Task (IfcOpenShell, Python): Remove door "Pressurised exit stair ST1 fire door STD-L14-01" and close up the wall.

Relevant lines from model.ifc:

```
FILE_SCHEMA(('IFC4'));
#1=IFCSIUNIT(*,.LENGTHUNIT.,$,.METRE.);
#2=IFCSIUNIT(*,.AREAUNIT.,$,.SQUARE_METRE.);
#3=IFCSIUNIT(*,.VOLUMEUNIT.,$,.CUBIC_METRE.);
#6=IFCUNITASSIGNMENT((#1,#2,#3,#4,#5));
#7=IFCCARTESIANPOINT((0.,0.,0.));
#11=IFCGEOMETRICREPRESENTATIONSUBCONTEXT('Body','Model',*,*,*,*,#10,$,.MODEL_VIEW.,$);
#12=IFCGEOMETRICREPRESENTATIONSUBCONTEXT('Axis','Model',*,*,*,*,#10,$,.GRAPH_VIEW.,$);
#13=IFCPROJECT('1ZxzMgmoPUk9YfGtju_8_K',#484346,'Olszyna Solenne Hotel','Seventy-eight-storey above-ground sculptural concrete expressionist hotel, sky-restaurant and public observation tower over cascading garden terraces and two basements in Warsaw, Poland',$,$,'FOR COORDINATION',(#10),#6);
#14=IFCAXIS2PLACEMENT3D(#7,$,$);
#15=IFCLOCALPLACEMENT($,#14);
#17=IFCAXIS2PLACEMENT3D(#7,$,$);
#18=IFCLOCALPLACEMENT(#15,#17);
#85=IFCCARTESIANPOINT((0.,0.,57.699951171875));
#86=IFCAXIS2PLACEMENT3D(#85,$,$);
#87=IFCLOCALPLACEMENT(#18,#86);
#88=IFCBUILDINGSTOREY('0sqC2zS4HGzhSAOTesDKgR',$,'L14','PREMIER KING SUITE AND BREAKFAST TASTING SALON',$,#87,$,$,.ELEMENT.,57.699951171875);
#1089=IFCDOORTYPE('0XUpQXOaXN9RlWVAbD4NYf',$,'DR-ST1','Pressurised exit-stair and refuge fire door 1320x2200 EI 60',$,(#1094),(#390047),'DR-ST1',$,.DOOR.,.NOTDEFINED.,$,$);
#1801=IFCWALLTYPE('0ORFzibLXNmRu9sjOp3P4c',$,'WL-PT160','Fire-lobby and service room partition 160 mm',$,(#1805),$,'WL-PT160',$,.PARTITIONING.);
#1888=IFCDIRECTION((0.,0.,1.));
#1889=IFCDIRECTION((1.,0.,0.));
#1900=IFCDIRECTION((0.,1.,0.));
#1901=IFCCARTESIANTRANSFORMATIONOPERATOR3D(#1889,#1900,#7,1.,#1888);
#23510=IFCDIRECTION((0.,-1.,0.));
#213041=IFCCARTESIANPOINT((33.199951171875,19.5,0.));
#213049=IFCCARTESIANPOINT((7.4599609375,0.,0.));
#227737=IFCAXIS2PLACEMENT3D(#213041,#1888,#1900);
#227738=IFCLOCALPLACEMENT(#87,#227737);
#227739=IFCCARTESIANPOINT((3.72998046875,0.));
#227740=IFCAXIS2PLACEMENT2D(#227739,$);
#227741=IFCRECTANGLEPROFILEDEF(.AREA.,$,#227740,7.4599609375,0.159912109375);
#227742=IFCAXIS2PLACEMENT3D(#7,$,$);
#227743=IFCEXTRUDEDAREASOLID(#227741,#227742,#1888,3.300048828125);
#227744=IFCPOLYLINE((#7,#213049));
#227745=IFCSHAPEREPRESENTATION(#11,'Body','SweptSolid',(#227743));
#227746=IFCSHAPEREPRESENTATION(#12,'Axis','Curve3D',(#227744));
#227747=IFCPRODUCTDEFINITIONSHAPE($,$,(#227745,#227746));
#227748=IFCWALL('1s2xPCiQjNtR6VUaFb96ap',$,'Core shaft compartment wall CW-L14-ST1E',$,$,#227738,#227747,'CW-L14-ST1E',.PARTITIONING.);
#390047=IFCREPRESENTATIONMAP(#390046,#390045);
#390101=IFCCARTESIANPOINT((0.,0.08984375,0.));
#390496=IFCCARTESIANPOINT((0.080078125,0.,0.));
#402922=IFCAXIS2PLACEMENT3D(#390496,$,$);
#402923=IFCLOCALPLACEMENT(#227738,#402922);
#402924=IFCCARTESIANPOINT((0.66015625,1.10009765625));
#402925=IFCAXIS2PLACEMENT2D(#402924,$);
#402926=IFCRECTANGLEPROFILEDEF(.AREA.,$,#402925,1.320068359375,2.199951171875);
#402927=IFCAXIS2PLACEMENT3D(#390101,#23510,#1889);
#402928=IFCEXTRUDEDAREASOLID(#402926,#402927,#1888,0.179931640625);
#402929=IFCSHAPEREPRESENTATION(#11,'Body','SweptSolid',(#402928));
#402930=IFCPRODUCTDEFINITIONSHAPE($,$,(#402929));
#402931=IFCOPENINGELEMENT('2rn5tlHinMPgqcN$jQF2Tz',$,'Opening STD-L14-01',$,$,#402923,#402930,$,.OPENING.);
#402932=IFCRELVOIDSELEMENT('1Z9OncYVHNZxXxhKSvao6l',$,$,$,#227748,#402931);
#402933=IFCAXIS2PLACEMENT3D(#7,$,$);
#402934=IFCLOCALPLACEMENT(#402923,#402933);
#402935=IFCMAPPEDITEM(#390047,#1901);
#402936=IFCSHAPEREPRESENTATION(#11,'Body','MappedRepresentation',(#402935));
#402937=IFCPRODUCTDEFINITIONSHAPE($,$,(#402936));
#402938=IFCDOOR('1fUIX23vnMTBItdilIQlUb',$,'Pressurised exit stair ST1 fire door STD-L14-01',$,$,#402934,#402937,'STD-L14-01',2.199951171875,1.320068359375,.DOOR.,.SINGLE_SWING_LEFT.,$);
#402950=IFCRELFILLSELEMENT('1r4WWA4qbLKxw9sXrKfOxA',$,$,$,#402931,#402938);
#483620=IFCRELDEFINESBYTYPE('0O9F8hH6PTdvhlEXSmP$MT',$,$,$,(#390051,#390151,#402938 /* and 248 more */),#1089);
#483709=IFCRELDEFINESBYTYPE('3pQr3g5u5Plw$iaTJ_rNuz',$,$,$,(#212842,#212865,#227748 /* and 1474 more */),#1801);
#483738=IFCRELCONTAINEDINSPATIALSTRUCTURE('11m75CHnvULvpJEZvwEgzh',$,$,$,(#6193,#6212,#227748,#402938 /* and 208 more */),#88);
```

```python
import ifcopenshell
import ifcopenshell.api.feature
import ifcopenshell.api.root
import ifcopenshell.geom
import ifcopenshell.util.shape

model = ifcopenshell.open("model.ifc")
settings = ifcopenshell.geom.settings()


def volume(element):
    """Net volume in cubic metres, openings subtracted."""
    shape = ifcopenshell.geom.create_shape(settings, element)
    return ifcopenshell.util.shape.get_volume(shape.geometry)


door = model.by_guid("1fUIX23vnMTBItdilIQlUb")
opening = door.FillsVoids[0].RelatingOpeningElement
wall = opening.VoidsElements[0].RelatingBuildingElement
before = volume(wall)

ifcopenshell.api.root.remove_product(model, product=door)
ifcopenshell.api.feature.remove_feature(model, feature=opening)

after = volume(wall)

print(f"wall volume {before:.3f} -> {after:.3f} m3")

model.write("model_updated.ifc")
```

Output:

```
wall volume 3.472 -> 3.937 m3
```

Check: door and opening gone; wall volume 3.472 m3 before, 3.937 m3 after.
